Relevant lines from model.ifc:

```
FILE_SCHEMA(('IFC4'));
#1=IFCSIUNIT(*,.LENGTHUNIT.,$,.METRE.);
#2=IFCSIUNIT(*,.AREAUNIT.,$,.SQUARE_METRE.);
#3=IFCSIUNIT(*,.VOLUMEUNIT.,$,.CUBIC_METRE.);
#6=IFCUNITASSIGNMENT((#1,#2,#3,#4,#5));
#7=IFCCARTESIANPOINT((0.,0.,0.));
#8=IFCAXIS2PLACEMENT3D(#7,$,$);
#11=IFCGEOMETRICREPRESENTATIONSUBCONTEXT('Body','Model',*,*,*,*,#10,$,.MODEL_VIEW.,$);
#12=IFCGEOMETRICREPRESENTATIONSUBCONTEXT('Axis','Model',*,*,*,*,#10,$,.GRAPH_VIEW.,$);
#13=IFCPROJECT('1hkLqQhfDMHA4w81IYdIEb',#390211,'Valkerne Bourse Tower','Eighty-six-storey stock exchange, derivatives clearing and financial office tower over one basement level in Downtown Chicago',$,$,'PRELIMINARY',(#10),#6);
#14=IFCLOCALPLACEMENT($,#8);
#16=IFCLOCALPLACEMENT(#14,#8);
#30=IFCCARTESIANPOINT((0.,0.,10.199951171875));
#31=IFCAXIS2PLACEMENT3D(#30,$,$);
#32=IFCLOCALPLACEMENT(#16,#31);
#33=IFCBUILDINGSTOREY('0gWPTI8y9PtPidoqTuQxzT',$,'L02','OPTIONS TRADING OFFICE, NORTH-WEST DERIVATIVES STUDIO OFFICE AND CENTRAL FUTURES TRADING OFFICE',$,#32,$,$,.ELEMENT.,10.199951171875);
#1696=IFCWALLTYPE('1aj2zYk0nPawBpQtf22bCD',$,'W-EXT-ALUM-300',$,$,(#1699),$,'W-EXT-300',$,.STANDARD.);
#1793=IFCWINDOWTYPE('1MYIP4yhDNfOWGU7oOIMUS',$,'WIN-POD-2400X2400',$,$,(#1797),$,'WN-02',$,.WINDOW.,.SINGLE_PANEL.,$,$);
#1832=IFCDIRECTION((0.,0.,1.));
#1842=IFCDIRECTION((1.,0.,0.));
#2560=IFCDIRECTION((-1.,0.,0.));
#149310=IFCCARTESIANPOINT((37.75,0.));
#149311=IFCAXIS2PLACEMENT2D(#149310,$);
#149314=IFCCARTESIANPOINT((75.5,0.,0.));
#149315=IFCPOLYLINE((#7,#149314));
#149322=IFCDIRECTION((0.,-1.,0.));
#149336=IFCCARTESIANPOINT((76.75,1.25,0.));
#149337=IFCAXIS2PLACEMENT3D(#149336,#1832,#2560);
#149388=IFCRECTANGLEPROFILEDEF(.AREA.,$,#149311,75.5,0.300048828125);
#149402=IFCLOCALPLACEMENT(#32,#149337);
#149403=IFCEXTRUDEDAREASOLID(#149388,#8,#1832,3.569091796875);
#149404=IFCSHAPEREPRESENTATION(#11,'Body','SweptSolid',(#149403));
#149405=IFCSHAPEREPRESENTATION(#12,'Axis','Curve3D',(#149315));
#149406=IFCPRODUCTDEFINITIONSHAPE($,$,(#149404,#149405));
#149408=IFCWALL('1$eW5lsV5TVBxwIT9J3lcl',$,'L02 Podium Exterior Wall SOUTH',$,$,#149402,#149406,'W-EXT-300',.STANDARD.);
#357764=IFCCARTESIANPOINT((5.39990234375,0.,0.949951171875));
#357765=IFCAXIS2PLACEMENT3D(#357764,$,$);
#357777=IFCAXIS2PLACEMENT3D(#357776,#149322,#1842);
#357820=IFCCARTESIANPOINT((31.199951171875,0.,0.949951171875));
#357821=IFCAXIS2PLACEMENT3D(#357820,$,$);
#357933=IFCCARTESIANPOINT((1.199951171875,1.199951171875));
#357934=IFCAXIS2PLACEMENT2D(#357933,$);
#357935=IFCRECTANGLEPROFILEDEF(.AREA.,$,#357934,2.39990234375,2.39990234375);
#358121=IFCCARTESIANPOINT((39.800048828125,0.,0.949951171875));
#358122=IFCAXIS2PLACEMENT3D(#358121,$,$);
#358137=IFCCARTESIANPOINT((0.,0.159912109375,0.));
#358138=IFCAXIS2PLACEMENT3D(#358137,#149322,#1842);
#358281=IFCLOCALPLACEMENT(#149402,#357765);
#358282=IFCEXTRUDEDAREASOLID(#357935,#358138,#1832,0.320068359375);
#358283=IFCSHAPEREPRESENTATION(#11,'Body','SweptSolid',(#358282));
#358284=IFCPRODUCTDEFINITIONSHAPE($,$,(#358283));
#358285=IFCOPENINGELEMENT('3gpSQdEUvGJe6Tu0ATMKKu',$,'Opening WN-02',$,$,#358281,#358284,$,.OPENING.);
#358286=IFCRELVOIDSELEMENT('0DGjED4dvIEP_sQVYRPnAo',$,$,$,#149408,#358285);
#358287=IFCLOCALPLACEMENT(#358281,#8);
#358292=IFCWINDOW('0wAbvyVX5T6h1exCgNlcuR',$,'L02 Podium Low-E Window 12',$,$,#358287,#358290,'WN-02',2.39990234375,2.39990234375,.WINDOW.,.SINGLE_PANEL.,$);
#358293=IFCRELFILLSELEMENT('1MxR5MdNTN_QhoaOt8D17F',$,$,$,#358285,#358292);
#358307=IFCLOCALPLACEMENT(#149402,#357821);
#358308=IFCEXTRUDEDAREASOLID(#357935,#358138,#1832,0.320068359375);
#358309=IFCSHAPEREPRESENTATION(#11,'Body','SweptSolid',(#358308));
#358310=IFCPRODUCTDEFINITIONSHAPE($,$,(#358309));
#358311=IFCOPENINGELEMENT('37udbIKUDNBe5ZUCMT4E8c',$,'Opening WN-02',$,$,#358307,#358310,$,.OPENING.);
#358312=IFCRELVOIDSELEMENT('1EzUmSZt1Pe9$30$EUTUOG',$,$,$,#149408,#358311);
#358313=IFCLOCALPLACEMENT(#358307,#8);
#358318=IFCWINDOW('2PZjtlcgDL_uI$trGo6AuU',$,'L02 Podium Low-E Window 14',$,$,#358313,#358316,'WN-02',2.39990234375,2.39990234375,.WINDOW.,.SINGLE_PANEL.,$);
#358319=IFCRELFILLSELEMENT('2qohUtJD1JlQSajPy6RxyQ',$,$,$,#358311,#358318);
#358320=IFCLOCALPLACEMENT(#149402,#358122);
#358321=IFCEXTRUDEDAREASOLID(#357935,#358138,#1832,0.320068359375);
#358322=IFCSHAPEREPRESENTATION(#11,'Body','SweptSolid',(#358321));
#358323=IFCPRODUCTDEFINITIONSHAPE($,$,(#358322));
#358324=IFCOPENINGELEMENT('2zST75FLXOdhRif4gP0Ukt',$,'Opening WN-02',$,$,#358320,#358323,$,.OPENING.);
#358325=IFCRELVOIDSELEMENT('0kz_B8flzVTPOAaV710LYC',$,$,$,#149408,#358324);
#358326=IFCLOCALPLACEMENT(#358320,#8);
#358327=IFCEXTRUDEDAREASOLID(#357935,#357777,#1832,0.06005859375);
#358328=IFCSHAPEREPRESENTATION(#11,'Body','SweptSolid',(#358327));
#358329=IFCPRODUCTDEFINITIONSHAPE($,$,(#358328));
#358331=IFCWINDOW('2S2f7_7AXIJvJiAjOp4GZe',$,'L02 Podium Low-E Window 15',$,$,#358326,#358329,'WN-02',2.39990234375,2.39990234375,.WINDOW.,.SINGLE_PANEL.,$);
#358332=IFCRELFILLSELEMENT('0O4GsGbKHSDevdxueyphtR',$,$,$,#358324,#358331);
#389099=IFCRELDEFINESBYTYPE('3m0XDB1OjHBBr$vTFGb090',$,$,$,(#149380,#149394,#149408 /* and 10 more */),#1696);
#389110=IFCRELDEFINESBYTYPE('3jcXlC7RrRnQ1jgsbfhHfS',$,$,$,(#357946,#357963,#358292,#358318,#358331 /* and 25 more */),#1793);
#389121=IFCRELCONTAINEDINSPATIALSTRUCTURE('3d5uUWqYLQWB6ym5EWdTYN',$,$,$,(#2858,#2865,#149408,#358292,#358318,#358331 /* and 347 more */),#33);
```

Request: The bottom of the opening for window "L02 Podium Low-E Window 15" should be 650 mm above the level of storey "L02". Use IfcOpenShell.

```python
import numpy as np
import ifcopenshell
import ifcopenshell.api.geometry
import ifcopenshell.geom
import ifcopenshell.util.element
import ifcopenshell.util.placement
import ifcopenshell.util.shape
import ifcopenshell.util.unit

model = ifcopenshell.open("model.ifc")
unit_scale = ifcopenshell.util.unit.calculate_unit_scale(model)

window = model.by_guid("2S2f7_7AXIJvJiAjOp4GZe")
opening = window.FillsVoids[0].RelatingOpeningElement
storey = ifcopenshell.util.element.get_container(window, ifc_class="IfcBuildingStorey")
level = ifcopenshell.util.placement.get_local_placement(storey.ObjectPlacement)[2, 3]

# The opening's origin need not be at the sill, so measure its lowest point.
shape = ifcopenshell.geom.create_shape(ifcopenshell.geom.settings(), opening)
bottom = ifcopenshell.util.shape.get_shape_bottom_elevation(shape, shape.geometry) / unit_scale
dz = level + 0.65 / unit_scale - bottom

shift = np.array([0.0, 0.0, dz])
# The window is placed relative to its opening, so it follows when the opening moves.
matrix = ifcopenshell.util.placement.get_local_placement(opening.ObjectPlacement)
matrix[:3, 3] += shift
ifcopenshell.api.geometry.edit_object_placement(
    model, product=opening, matrix=matrix, is_si=False, should_transform_children=True
)

print(f"moved by {dz * unit_scale:+.3f} m")

model.write("model-out.ifc")
```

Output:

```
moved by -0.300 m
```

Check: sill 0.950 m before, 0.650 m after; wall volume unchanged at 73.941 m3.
